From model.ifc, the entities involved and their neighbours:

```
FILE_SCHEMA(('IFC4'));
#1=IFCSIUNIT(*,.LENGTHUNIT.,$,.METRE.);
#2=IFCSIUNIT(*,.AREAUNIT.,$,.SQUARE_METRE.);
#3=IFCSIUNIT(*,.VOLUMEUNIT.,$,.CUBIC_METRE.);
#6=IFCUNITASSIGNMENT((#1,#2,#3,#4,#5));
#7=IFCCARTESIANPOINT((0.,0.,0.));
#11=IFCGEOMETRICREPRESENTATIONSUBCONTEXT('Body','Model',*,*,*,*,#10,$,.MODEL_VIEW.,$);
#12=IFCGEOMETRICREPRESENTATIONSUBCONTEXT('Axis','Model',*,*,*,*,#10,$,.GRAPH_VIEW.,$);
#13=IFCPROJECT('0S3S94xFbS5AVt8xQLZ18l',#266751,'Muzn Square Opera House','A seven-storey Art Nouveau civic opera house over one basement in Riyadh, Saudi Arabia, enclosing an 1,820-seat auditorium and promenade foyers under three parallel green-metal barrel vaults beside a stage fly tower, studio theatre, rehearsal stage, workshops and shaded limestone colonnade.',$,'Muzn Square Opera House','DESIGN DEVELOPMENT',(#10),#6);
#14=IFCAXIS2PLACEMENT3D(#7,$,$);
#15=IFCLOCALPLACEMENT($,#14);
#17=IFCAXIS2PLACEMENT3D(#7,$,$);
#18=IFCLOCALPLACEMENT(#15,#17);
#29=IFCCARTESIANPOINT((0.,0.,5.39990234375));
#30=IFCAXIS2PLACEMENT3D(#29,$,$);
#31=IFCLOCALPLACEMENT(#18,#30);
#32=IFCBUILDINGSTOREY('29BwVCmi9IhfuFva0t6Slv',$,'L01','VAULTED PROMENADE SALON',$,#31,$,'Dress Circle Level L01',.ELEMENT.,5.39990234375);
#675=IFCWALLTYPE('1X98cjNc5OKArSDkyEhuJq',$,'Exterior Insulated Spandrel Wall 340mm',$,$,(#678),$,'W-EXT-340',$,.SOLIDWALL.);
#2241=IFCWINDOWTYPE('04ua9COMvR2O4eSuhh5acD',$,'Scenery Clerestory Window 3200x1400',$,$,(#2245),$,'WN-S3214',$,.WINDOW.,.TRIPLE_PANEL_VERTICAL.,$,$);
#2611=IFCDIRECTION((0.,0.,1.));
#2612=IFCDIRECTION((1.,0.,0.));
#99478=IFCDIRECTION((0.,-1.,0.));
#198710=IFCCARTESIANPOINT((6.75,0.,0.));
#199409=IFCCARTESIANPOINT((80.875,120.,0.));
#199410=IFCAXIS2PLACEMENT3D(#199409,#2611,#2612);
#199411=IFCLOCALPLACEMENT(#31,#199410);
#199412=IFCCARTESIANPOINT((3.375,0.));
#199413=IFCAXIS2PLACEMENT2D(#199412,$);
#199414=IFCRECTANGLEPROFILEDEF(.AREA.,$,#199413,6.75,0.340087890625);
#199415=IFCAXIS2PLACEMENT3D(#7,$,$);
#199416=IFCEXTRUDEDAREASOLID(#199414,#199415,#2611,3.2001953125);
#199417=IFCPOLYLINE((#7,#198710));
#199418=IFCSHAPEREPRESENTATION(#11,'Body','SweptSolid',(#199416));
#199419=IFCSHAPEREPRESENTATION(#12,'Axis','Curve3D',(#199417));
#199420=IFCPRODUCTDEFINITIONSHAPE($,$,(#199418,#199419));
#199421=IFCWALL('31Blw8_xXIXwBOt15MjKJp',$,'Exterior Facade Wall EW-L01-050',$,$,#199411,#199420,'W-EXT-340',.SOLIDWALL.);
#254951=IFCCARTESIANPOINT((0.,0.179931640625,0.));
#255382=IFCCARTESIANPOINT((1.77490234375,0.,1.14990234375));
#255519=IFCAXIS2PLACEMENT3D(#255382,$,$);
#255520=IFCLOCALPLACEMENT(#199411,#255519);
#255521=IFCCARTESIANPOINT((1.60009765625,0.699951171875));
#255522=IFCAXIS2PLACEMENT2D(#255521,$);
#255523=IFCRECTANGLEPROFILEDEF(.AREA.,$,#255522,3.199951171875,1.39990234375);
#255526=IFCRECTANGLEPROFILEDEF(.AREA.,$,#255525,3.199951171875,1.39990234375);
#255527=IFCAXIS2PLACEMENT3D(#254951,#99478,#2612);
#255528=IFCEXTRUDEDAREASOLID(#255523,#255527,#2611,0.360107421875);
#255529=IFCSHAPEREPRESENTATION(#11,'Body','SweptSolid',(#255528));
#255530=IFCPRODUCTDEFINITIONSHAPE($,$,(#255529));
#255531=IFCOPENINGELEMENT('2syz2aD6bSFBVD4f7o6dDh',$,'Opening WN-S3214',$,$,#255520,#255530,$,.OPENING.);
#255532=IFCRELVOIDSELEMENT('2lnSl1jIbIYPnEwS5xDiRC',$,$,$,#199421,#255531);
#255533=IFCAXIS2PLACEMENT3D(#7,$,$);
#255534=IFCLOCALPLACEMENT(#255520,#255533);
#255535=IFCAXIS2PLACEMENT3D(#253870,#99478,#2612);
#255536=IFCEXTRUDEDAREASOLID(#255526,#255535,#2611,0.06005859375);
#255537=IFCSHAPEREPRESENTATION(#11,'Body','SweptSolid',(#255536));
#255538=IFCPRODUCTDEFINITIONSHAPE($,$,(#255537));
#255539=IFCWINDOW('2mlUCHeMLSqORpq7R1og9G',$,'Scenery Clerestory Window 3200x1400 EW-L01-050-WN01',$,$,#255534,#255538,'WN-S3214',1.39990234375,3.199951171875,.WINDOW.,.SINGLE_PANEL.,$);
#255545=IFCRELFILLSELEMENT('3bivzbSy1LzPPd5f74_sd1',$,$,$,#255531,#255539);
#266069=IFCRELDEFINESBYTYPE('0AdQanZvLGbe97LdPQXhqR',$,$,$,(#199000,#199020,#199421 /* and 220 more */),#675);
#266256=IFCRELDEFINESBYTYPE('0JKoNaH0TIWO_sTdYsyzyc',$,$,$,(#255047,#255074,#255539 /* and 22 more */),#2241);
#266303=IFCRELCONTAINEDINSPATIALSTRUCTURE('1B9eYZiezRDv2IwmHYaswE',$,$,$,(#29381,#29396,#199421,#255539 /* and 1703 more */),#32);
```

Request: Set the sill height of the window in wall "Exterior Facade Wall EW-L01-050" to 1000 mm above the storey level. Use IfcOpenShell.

```python
import numpy as np
import ifcopenshell
import ifcopenshell.api.geometry
import ifcopenshell.geom
import ifcopenshell.util.element
import ifcopenshell.util.placement
import ifcopenshell.util.shape
import ifcopenshell.util.unit

model = ifcopenshell.open("model.ifc")
unit_scale = ifcopenshell.util.unit.calculate_unit_scale(model)

window = model.by_guid("2mlUCHeMLSqORpq7R1og9G")
opening = window.FillsVoids[0].RelatingOpeningElement
storey = ifcopenshell.util.element.get_container(window, ifc_class="IfcBuildingStorey")
level = ifcopenshell.util.placement.get_local_placement(storey.ObjectPlacement)[2, 3]

# The opening's origin need not be at the sill, so measure its lowest point.
shape = ifcopenshell.geom.create_shape(ifcopenshell.geom.settings(), opening)
bottom = ifcopenshell.util.shape.get_shape_bottom_elevation(shape, shape.geometry) / unit_scale
dz = level + 1.0 - bottom

shift = np.array([0.0, 0.0, dz])
# The window is placed relative to its opening, so it follows when the opening moves.
matrix = ifcopenshell.util.placement.get_local_placement(opening.ObjectPlacement)
matrix[:3, 3] += shift
ifcopenshell.api.geometry.edit_object_placement(
    model, product=opening, matrix=matrix, is_si=False, should_transform_children=True
)

print(f"moved by {dz * unit_scale:+.3f} m")

model.write("model_edited.ifc")
```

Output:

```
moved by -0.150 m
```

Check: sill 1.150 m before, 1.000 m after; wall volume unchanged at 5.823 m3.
